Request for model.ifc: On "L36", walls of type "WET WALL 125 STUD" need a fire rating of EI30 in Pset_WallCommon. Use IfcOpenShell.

First a look at what the model holds.

```python
import ifcopenshell
import ifcopenshell.util.element

model = ifcopenshell.open("model.ifc")
print(model.schema)
storey = next(s for s in model.by_type("IfcBuildingStorey") if s.Name == "L36")
walls = [e for e in ifcopenshell.util.element.get_decomposition(storey) if e.is_a("IfcWall")]
seen = {}
for e in walls:
    element_type = ifcopenshell.util.element.get_type(e)
    key = (element_type.Name if element_type != e and element_type else None, ifcopenshell.util.element.get_pset(e, "Pset_WallCommon", "FireRating"))
    seen[key] = seen.get(key, 0) + 1
for (name, value), count in sorted(seen.items(), key=str):
    print(count, "x", name, "|", value)
```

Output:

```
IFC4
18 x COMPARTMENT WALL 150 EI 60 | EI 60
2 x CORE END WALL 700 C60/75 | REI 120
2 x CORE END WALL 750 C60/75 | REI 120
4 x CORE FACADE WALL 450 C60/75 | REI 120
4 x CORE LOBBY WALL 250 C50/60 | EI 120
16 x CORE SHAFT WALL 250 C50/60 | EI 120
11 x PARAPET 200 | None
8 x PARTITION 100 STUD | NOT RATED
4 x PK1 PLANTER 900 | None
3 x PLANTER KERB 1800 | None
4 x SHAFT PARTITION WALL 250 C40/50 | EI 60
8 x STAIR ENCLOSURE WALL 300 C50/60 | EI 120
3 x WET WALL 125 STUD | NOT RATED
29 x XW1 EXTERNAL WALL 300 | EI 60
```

```python
import ifcopenshell
import ifcopenshell.api.pset
import ifcopenshell.util.element

model = ifcopenshell.open("model.ifc")

storey = next(s for s in model.by_type("IfcBuildingStorey") if s.Name == "L36")
walls = [e for e in ifcopenshell.util.element.get_decomposition(storey) if e.is_a("IfcWall")]

count = 0
for e in walls:
    element_type = ifcopenshell.util.element.get_type(e)
    if element_type in (None, e) or element_type.Name != "WET WALL 125 STUD":
        continue
    found = ifcopenshell.util.element.get_pset(e, "Pset_WallCommon", should_inherit=False)
    if found:
        pset = model.by_id(found["id"])
        if len(ifcopenshell.util.element.get_elements_by_pset(pset)) > 1:
            pset = ifcopenshell.api.pset.unshare_pset(model, products=[e], pset=pset)[0]
    else:
        pset = ifcopenshell.api.pset.add_pset(model, product=e, name="Pset_WallCommon")
    ifcopenshell.api.pset.edit_pset(model, pset=pset, properties={"FireRating": "EI30"})
    count += 1

print(count, "walls updated")

model.write("model_edited.ifc")
```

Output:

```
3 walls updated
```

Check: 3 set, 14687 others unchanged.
